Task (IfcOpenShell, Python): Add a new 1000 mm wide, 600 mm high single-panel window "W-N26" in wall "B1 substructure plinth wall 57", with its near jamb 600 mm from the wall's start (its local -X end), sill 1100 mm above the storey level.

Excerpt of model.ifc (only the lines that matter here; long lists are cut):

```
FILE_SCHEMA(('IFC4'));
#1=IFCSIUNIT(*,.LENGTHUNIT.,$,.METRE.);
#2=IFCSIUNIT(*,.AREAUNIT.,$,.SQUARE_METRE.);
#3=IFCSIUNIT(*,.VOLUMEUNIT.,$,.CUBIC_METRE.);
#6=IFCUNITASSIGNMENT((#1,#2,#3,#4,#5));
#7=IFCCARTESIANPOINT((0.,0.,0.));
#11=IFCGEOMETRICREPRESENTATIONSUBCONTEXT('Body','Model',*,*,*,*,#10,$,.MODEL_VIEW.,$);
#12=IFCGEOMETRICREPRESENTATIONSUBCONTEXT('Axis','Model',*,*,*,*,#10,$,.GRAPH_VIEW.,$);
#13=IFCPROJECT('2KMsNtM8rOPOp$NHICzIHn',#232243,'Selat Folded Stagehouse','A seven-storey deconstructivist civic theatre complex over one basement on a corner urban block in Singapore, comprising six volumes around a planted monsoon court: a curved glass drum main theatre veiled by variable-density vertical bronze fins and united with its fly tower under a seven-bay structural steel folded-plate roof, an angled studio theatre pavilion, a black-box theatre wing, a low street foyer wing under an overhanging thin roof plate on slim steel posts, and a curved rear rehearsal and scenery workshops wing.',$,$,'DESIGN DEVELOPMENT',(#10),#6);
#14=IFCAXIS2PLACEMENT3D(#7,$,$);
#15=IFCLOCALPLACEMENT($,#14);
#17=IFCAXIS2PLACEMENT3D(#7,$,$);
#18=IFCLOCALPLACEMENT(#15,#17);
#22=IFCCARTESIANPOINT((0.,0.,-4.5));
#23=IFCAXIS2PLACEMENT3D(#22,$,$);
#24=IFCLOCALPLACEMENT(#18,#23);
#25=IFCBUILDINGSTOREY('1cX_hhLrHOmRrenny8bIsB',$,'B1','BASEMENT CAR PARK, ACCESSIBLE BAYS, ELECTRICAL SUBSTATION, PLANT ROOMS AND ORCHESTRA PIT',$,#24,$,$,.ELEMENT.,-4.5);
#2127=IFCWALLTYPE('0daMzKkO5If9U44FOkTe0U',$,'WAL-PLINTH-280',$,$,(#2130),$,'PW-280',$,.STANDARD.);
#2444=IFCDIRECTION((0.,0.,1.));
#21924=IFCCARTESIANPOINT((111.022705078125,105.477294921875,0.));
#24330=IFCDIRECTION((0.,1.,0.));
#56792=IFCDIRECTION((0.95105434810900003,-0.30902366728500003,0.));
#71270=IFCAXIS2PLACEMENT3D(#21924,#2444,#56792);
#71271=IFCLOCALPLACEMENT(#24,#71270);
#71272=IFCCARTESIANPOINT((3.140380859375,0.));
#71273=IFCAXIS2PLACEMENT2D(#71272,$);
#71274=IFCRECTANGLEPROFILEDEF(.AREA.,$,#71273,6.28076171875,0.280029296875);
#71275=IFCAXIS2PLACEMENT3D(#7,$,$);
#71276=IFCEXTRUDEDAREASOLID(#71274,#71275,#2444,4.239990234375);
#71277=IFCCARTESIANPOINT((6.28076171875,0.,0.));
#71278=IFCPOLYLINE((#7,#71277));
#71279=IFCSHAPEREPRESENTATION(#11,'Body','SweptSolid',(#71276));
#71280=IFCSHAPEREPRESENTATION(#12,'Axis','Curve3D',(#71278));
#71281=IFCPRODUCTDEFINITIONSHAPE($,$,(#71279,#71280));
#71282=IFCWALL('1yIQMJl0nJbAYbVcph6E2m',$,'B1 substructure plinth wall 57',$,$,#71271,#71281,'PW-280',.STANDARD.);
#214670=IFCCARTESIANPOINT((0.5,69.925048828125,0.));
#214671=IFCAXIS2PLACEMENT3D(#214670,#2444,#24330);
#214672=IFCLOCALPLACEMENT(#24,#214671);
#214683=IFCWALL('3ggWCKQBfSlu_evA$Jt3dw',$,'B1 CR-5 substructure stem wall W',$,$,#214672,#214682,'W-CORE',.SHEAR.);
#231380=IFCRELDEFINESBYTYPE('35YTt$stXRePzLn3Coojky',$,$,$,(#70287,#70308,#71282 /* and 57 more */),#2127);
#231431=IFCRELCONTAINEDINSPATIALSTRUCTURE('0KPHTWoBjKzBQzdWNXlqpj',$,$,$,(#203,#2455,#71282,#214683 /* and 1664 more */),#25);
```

```python
import numpy as np
import ifcopenshell
import ifcopenshell.api.feature
import ifcopenshell.api.geometry
import ifcopenshell.api.root
import ifcopenshell.api.spatial
import ifcopenshell.geom
import ifcopenshell.util.element
import ifcopenshell.util.placement
import ifcopenshell.util.representation
import ifcopenshell.util.shape
import ifcopenshell.util.unit

model = ifcopenshell.open("model.ifc")
unit_scale = ifcopenshell.util.unit.calculate_unit_scale(model)
settings = ifcopenshell.geom.settings()


def volume(element):
    """Net volume in cubic metres, openings subtracted."""
    shape = ifcopenshell.geom.create_shape(settings, element)
    return ifcopenshell.util.shape.get_volume(shape.geometry)


wall = model.by_guid("1yIQMJl0nJbAYbVcph6E2m")
storey = ifcopenshell.util.element.get_container(wall, ifc_class="IfcBuildingStorey")
context = ifcopenshell.util.representation.get_context(model, "Model", "Body", "MODEL_VIEW")
before = volume(wall)

width, height, from_end, sill = 1, 0.6, 0.6, 1.1  # metres

# The wall runs along its own X axis, and the end named is its -X end.
wall_shape = ifcopenshell.geom.create_shape(settings, wall)
x, y, z = ifcopenshell.util.shape.get_vertices(wall_shape.geometry).T
start = x.min() + from_end
face, thickness = float(y.min()), float(y.max() - y.min())
wall_matrix = ifcopenshell.util.placement.get_local_placement(wall.ObjectPlacement)
level = ifcopenshell.util.placement.get_local_placement(storey.ObjectPlacement)[2, 3]


def in_wall(x, y):
    """Placement at x, y metres in the wall's axes, at sill height."""
    matrix = wall_matrix.copy()
    matrix[:, 3] = wall_matrix @ np.array([x / unit_scale, y / unit_scale, 0.0, 1.0])
    matrix[2, 3] = level + sill / unit_scale
    return matrix


# Opening: a box that overshoots both wall faces by 50 mm.
opening = ifcopenshell.api.root.create_entity(model, ifc_class="IfcOpeningElement", predefined_type="OPENING")
box = ifcopenshell.api.geometry.add_wall_representation(
    model, context=context, length=width, height=height, thickness=thickness + 0.1
)
ifcopenshell.api.geometry.assign_representation(model, product=opening, representation=box)
ifcopenshell.api.geometry.edit_object_placement(model, product=opening, matrix=in_wall(start, face - 0.05), is_si=False)
ifcopenshell.api.feature.add_feature(model, feature=opening, element=wall)

window = ifcopenshell.api.root.create_entity(model, ifc_class="IfcWindow", name="W-N26", predefined_type="WINDOW")
window.OverallWidth, window.OverallHeight = width / unit_scale, height / unit_scale
window.PartitioningType = "SINGLE_PANEL"
body = ifcopenshell.api.geometry.add_window_representation(
    model,
    context=context,
    overall_width=window.OverallWidth,
    overall_height=window.OverallHeight,
    partition_type="SINGLE_PANEL",
)
ifcopenshell.api.geometry.assign_representation(model, product=window, representation=body)
ifcopenshell.api.spatial.assign_container(model, products=[window], relating_structure=storey)
ifcopenshell.api.feature.add_filling(model, opening=opening, element=window)

# Centre the window in the wall's thickness.
ifcopenshell.api.geometry.edit_object_placement(model, product=window, matrix=in_wall(start, face), is_si=False)
window_shape = ifcopenshell.geom.create_shape(settings, window)
depth = ifcopenshell.util.shape.get_vertices(window_shape.geometry)[:, 1]
offset = face + thickness / 2 - (depth.min() + depth.max()) / 2
ifcopenshell.api.geometry.edit_object_placement(model, product=window, matrix=in_wall(start, offset), is_si=False)

after = volume(wall)

print(f"wall volume {before:.3f} -> {after:.3f} m3")

model.write("model-out.ifc")
```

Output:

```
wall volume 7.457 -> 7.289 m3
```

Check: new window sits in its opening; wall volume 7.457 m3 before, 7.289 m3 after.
